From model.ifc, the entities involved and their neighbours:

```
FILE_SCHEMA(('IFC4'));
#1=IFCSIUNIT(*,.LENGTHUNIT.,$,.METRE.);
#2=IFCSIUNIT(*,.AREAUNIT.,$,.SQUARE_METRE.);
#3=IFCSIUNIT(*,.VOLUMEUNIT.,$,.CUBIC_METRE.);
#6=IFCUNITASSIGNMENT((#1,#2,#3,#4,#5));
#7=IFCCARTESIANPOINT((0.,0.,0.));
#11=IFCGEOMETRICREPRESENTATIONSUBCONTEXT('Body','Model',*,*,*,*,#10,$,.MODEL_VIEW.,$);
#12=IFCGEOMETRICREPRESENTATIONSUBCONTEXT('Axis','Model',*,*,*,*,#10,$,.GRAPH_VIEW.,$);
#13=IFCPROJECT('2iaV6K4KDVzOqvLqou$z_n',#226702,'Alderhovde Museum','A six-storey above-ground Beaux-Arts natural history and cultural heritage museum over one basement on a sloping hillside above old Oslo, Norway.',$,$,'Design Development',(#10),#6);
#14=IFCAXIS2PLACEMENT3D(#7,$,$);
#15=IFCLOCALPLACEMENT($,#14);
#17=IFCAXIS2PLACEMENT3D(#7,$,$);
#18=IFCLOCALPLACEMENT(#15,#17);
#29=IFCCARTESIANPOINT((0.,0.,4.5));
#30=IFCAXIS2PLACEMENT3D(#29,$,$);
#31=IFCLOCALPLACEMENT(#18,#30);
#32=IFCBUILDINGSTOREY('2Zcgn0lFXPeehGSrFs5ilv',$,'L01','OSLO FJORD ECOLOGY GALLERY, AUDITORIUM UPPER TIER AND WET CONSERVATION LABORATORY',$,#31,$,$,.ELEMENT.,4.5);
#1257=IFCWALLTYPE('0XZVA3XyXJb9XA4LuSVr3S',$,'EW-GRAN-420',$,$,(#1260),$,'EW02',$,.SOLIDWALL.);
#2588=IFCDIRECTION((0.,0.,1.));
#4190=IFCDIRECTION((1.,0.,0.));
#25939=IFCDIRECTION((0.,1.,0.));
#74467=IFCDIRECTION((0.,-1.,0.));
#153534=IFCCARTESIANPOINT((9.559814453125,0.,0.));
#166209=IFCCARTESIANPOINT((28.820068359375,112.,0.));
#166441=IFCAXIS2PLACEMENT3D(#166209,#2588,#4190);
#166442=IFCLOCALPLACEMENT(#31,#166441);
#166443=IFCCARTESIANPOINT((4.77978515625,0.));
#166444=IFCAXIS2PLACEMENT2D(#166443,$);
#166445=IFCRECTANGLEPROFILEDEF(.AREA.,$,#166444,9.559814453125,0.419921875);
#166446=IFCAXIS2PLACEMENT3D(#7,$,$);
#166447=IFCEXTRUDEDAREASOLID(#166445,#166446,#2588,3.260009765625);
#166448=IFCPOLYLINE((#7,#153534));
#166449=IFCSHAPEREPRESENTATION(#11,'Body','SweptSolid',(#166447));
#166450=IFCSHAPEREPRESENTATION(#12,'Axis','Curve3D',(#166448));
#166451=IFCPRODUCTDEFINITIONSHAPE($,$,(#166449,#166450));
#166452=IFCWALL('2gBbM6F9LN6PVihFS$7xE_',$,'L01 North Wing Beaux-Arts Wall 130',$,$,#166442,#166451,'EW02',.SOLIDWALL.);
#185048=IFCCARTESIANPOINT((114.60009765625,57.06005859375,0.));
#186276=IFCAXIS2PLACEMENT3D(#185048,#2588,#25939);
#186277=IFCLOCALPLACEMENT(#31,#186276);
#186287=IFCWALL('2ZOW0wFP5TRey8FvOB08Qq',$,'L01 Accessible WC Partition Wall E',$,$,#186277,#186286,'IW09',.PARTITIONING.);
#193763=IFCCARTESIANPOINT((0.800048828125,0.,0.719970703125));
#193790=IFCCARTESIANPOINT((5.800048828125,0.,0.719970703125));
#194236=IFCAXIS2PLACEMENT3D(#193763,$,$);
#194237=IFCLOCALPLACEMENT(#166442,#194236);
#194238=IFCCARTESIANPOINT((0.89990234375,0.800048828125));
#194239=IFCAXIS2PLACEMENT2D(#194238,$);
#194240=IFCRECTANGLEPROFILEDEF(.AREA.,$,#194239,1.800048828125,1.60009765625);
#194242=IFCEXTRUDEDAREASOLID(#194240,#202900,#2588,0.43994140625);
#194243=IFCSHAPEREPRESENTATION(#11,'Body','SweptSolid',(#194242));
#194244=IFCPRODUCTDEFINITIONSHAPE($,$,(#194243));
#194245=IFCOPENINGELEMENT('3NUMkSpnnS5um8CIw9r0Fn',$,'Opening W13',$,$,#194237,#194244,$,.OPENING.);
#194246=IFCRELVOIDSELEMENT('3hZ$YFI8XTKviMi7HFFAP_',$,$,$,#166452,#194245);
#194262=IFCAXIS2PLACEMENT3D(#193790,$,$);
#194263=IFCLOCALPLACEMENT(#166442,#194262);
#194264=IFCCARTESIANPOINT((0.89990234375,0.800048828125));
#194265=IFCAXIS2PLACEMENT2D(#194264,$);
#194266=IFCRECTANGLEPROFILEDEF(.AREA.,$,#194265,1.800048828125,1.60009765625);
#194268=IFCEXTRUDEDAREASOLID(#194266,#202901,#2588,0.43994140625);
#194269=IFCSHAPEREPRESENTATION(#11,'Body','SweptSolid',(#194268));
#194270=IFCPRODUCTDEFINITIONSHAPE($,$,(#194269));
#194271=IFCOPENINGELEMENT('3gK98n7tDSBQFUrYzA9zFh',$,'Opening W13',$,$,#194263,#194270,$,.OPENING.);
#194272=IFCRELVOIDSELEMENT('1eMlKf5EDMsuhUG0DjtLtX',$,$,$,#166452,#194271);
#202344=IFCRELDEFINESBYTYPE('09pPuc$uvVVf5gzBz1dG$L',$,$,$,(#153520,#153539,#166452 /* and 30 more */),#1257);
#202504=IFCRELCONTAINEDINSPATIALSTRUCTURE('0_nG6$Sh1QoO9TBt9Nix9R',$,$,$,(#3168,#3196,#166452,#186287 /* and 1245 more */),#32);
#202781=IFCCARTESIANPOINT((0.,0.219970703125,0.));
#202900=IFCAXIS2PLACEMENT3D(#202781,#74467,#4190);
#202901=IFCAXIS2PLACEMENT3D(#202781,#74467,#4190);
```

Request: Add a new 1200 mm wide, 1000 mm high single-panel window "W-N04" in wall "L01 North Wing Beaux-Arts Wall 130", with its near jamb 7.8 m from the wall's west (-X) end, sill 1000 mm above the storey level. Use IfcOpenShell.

```python
import numpy as np
import ifcopenshell
import ifcopenshell.api.feature
import ifcopenshell.api.geometry
import ifcopenshell.api.root
import ifcopenshell.api.spatial
import ifcopenshell.geom
import ifcopenshell.util.element
import ifcopenshell.util.placement
import ifcopenshell.util.representation
import ifcopenshell.util.shape
import ifcopenshell.util.unit

model = ifcopenshell.open("model.ifc")
unit_scale = ifcopenshell.util.unit.calculate_unit_scale(model)
settings = ifcopenshell.geom.settings()


def volume(element):
    """Net volume in cubic metres, openings subtracted."""
    shape = ifcopenshell.geom.create_shape(settings, element)
    return ifcopenshell.util.shape.get_volume(shape.geometry)


wall = model.by_id(166452)
storey = ifcopenshell.util.element.get_container(wall, ifc_class="IfcBuildingStorey")
context = ifcopenshell.util.representation.get_context(model, "Model", "Body", "MODEL_VIEW")
before = volume(wall)

width, height, from_end, sill = 1.2, 1, 7.8, 1  # metres

# The wall runs along its own X axis, and the end named is its -X end.
wall_shape = ifcopenshell.geom.create_shape(settings, wall)
x, y, z = ifcopenshell.util.shape.get_vertices(wall_shape.geometry).T
start = x.min() + from_end
face, thickness = float(y.min()), float(y.max() - y.min())
wall_matrix = ifcopenshell.util.placement.get_local_placement(wall.ObjectPlacement)
level = ifcopenshell.util.placement.get_local_placement(storey.ObjectPlacement)[2, 3]


def in_wall(x, y):
    """Placement at x, y metres in the wall's axes, at sill height."""
    matrix = wall_matrix.copy()
    matrix[:, 3] = wall_matrix @ np.array([x / unit_scale, y / unit_scale, 0.0, 1.0])
    matrix[2, 3] = level + sill / unit_scale
    return matrix


# Opening: a box that overshoots both wall faces by 50 mm.
opening = ifcopenshell.api.root.create_entity(model, ifc_class="IfcOpeningElement", predefined_type="OPENING")
box = ifcopenshell.api.geometry.add_wall_representation(
    model, context=context, length=width, height=height, thickness=thickness + 0.1
)
ifcopenshell.api.geometry.assign_representation(model, product=opening, representation=box)
ifcopenshell.api.geometry.edit_object_placement(model, product=opening, matrix=in_wall(start, face - 0.05), is_si=False)
ifcopenshell.api.feature.add_feature(model, feature=opening, element=wall)

window = ifcopenshell.api.root.create_entity(model, ifc_class="IfcWindow", name="W-N04", predefined_type="WINDOW")
window.OverallWidth, window.OverallHeight = width / unit_scale, height / unit_scale
window.PartitioningType = "SINGLE_PANEL"
body = ifcopenshell.api.geometry.add_window_representation(
    model,
    context=context,
    overall_width=window.OverallWidth,
    overall_height=window.OverallHeight,
    partition_type="SINGLE_PANEL",
)
ifcopenshell.api.geometry.assign_representation(model, product=window, representation=body)
ifcopenshell.api.spatial.assign_container(model, products=[window], relating_structure=storey)
ifcopenshell.api.feature.add_filling(model, opening=opening, element=window)

# Centre the window in the wall's thickness.
ifcopenshell.api.geometry.edit_object_placement(model, product=window, matrix=in_wall(start, face), is_si=False)
window_shape = ifcopenshell.geom.create_shape(settings, window)
depth = ifcopenshell.util.shape.get_vertices(window_shape.geometry)[:, 1]
offset = face + thickness / 2 - (depth.min() + depth.max()) / 2
ifcopenshell.api.geometry.edit_object_placement(model, product=window, matrix=in_wall(start, offset), is_si=False)

after = volume(wall)

print(f"wall volume {before:.3f} -> {after:.3f} m3")

model.write("model_updated.ifc")
```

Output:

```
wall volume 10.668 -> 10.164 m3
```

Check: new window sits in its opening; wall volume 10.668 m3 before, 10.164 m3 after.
